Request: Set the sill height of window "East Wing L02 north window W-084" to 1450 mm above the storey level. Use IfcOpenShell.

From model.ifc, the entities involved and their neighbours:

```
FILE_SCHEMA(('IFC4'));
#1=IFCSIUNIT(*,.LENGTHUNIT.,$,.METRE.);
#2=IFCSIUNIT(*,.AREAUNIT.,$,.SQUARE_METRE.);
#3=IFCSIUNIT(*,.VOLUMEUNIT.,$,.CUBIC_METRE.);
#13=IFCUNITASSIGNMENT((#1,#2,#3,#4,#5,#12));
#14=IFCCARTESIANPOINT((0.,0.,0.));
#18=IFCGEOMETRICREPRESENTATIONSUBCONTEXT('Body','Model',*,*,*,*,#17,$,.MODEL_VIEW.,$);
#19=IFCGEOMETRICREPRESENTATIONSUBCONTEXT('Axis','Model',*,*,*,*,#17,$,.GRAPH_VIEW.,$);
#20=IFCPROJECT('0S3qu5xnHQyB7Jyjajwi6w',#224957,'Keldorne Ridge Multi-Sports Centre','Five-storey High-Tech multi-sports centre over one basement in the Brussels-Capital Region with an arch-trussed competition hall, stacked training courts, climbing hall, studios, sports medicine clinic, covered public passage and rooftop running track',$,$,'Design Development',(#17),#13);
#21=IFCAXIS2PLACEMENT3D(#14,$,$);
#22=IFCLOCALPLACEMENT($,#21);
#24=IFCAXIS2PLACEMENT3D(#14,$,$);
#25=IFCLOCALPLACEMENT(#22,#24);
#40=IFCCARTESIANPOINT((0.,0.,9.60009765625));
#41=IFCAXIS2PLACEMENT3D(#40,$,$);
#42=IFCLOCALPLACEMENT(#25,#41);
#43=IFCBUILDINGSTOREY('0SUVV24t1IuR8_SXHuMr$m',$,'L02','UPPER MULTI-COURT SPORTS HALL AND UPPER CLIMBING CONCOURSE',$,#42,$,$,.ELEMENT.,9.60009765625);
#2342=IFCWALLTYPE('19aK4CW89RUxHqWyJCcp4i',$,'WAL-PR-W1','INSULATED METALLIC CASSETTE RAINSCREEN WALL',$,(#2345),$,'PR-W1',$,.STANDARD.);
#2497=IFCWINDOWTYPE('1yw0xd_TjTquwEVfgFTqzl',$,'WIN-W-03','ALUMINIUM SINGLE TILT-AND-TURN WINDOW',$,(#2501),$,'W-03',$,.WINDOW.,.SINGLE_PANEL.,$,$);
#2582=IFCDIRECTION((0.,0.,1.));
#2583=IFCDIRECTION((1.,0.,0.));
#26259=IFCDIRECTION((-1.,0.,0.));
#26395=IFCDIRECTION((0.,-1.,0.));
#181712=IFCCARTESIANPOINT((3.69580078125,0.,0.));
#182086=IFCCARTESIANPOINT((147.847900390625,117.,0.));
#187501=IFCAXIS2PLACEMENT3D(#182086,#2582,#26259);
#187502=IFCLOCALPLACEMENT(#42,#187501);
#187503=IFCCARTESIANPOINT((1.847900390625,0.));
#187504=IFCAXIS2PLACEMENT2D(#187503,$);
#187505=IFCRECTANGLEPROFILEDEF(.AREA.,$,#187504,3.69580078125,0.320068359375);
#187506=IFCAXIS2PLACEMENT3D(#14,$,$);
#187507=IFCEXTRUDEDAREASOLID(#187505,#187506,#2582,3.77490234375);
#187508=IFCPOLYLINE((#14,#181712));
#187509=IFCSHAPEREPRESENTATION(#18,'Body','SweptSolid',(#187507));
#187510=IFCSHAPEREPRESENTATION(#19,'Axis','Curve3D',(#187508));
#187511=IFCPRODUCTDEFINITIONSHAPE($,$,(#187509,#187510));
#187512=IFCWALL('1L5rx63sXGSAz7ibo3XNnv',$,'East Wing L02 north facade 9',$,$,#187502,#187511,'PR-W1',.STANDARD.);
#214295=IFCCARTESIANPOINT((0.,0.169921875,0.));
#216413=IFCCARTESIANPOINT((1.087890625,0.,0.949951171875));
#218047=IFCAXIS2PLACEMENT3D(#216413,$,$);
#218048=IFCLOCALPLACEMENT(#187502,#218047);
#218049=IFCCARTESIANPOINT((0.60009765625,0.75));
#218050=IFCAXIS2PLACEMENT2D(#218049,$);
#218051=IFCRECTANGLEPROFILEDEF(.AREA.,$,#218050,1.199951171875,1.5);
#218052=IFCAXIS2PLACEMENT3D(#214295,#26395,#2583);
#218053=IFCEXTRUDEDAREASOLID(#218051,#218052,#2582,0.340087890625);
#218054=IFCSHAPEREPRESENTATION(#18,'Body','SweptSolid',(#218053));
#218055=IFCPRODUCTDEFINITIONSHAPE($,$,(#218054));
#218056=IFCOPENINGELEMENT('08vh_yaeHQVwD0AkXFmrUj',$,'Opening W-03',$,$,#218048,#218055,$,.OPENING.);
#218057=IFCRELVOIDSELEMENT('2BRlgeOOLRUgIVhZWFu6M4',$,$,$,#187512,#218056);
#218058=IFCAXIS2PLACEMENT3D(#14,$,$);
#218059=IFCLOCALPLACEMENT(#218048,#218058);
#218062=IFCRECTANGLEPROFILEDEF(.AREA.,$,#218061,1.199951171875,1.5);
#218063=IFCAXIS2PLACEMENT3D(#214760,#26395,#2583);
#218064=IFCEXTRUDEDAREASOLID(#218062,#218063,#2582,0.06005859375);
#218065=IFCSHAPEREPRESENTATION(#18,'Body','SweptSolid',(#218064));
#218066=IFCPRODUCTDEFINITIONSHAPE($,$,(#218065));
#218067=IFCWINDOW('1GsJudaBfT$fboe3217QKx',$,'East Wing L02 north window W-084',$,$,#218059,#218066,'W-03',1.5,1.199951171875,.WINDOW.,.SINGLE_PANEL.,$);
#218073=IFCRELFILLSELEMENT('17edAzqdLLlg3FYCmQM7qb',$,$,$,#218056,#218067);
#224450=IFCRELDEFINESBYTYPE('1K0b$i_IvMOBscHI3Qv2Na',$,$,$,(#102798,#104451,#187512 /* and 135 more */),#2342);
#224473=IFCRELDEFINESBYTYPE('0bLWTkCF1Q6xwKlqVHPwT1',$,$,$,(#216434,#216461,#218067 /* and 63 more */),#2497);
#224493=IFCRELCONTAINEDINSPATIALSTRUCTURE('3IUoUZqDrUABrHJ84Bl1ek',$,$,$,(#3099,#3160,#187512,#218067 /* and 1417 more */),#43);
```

```python
import numpy as np
import ifcopenshell
import ifcopenshell.api.geometry
import ifcopenshell.geom
import ifcopenshell.util.element
import ifcopenshell.util.placement
import ifcopenshell.util.shape
import ifcopenshell.util.unit

model = ifcopenshell.open("model.ifc")
unit_scale = ifcopenshell.util.unit.calculate_unit_scale(model)

window = model.by_id(218067)
opening = window.FillsVoids[0].RelatingOpeningElement
storey = ifcopenshell.util.element.get_container(window, ifc_class="IfcBuildingStorey")
level = ifcopenshell.util.placement.get_local_placement(storey.ObjectPlacement)[2, 3]

# The opening's origin need not be at the sill, so measure its lowest point.
shape = ifcopenshell.geom.create_shape(ifcopenshell.geom.settings(), opening)
bottom = ifcopenshell.util.shape.get_shape_bottom_elevation(shape, shape.geometry) / unit_scale
dz = level + 1.45 / unit_scale - bottom

shift = np.array([0.0, 0.0, dz])
# The window is placed relative to its opening, so it follows when the opening moves.
matrix = ifcopenshell.util.placement.get_local_placement(opening.ObjectPlacement)
matrix[:3, 3] += shift
ifcopenshell.api.geometry.edit_object_placement(
    model, product=opening, matrix=matrix, is_si=False, should_transform_children=True
)

print(f"moved by {dz * unit_scale:+.3f} m")

model.write("model_v2.ifc")
```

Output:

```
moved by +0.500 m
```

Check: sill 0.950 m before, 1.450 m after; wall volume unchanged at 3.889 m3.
